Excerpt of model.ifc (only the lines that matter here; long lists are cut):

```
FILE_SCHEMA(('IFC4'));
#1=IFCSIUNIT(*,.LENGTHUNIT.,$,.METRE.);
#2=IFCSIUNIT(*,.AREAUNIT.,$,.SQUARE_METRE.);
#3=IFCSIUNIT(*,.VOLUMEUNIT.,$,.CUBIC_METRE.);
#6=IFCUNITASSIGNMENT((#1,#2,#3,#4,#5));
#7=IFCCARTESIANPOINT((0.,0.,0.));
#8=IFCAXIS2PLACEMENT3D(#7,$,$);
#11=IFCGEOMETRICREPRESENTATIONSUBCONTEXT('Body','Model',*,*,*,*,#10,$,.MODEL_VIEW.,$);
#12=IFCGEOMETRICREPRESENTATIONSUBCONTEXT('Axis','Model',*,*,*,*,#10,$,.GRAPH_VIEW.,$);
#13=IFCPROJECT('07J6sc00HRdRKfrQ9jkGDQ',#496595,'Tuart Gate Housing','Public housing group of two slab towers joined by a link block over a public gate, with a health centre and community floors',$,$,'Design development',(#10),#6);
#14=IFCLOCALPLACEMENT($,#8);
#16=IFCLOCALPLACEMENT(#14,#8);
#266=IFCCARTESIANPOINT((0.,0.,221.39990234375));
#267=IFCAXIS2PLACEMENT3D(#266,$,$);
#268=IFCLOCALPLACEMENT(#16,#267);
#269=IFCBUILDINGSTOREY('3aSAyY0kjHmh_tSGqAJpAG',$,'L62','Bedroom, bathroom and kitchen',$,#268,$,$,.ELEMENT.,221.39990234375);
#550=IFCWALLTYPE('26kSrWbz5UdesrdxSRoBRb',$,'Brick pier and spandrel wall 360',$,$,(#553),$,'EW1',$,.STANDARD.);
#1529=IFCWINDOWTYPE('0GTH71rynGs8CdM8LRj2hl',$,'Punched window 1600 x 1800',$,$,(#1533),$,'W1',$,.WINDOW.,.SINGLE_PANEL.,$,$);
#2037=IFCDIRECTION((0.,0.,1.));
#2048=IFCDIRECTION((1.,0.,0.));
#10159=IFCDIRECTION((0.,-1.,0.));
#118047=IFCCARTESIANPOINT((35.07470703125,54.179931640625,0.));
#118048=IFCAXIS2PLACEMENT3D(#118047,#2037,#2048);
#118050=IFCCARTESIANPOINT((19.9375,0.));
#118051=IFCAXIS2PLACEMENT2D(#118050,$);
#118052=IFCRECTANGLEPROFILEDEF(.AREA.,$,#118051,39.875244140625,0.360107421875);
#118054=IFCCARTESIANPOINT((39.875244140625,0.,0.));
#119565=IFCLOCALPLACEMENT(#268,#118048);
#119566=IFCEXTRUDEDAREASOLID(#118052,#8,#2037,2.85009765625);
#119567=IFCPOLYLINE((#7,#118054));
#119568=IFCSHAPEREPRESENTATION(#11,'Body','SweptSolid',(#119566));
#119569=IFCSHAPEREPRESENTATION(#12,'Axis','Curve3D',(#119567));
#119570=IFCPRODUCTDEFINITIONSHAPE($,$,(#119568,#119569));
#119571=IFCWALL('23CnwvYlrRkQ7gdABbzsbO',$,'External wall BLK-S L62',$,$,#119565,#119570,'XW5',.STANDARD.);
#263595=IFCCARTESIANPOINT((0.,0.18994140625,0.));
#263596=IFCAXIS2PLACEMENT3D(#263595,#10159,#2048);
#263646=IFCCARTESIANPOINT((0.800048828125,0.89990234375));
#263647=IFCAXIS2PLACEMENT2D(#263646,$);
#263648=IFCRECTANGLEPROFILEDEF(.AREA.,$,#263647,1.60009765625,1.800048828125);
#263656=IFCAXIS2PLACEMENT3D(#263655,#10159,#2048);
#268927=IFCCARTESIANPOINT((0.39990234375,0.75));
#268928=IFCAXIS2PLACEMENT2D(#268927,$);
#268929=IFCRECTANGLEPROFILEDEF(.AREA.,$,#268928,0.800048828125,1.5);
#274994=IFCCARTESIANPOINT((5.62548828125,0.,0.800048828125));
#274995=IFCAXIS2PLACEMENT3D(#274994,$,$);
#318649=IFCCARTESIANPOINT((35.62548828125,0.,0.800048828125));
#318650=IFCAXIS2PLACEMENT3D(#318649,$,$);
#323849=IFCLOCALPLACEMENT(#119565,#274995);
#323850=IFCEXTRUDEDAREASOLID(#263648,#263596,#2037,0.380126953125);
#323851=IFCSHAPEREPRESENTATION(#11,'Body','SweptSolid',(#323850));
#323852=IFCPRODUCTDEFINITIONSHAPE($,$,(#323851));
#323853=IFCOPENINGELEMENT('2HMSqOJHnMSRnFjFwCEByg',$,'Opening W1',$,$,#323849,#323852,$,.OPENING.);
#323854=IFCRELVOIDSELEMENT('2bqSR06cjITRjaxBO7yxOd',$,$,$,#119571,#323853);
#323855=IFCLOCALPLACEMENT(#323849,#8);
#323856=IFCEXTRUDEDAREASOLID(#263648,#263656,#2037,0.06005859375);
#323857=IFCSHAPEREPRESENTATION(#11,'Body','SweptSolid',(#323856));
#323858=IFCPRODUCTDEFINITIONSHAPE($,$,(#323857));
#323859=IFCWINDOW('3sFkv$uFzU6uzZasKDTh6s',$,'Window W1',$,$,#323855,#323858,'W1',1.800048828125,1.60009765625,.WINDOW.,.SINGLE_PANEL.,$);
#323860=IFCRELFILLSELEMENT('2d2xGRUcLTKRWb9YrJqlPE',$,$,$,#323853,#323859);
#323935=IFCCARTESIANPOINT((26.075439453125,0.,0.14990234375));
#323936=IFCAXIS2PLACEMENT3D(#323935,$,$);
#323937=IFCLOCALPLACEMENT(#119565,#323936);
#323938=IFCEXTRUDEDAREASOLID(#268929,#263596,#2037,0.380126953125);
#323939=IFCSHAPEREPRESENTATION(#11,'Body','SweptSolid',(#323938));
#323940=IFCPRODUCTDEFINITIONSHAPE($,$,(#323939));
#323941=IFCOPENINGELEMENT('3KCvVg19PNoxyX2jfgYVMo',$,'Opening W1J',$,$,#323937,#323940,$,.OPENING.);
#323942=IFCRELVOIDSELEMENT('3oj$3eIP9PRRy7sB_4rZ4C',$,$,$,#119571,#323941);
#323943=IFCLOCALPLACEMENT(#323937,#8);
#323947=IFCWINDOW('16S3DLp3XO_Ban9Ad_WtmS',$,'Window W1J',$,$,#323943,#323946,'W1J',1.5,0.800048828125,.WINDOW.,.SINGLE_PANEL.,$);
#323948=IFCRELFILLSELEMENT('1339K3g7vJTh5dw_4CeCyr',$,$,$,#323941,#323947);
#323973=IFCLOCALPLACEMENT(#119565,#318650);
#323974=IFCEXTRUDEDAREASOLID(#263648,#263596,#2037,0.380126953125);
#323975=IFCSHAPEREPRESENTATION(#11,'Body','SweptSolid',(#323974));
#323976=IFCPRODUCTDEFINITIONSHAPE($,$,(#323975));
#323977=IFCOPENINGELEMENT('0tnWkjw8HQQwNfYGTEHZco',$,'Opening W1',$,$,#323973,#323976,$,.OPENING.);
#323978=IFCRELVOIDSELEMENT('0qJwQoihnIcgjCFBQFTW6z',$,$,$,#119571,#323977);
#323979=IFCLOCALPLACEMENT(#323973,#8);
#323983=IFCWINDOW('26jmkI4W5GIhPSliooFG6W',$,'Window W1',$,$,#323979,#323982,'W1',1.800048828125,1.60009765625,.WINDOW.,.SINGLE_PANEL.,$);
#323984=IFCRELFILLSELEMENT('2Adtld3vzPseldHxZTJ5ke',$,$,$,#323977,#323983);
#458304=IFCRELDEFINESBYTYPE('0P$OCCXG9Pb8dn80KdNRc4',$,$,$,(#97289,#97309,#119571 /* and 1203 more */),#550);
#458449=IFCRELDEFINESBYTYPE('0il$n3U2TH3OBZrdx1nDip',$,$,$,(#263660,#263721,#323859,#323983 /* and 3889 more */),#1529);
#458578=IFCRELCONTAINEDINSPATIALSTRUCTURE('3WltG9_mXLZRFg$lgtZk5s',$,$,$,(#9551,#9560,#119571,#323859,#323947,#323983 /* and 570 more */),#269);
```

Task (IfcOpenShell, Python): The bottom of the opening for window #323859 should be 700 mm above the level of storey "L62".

```python
import numpy as np
import ifcopenshell
import ifcopenshell.api.geometry
import ifcopenshell.geom
import ifcopenshell.util.element
import ifcopenshell.util.placement
import ifcopenshell.util.shape
import ifcopenshell.util.unit

model = ifcopenshell.open("model.ifc")
unit_scale = ifcopenshell.util.unit.calculate_unit_scale(model)

window = model.by_guid("3sFkv$uFzU6uzZasKDTh6s")
opening = window.FillsVoids[0].RelatingOpeningElement
storey = ifcopenshell.util.element.get_container(window, ifc_class="IfcBuildingStorey")
level = ifcopenshell.util.placement.get_local_placement(storey.ObjectPlacement)[2, 3]

# The opening's origin need not be at the sill, so measure its lowest point.
shape = ifcopenshell.geom.create_shape(ifcopenshell.geom.settings(), opening)
bottom = ifcopenshell.util.shape.get_shape_bottom_elevation(shape, shape.geometry) / unit_scale
dz = level + 0.7 / unit_scale - bottom

shift = np.array([0.0, 0.0, dz])
# The window is placed relative to its opening, so it follows when the opening moves.
matrix = ifcopenshell.util.placement.get_local_placement(opening.ObjectPlacement)
matrix[:3, 3] += shift
ifcopenshell.api.geometry.edit_object_placement(
    model, product=opening, matrix=matrix, is_si=False, should_transform_children=True
)

print(f"moved by {dz * unit_scale:+.3f} m")

model.write("model_updated.ifc")
```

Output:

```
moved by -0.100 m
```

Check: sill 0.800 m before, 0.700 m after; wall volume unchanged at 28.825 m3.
